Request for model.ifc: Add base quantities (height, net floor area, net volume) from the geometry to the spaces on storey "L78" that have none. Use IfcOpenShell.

First a look at what the model holds.

```python
import ifcopenshell
import ifcopenshell.util.element
import ifcopenshell.util.unit

model = ifcopenshell.open("model.ifc")
print(model.schema)
for unit_type in ("LENGTHUNIT", "AREAUNIT", "VOLUMEUNIT"):
    print(unit_type, ifcopenshell.util.unit.calculate_unit_scale(model, unit_type))
storey = next(s for s in model.by_type("IfcBuildingStorey") if s.Name == "L78")
spaces = [e for e in ifcopenshell.util.element.get_decomposition(storey) if e.is_a("IfcSpace")]
for e in sorted(spaces, key=lambda e: e.id()):
    print(e.id(), e.is_a(), e.Name, list(ifcopenshell.util.element.get_psets(e, qtos_only=True)), sep=" | ")
```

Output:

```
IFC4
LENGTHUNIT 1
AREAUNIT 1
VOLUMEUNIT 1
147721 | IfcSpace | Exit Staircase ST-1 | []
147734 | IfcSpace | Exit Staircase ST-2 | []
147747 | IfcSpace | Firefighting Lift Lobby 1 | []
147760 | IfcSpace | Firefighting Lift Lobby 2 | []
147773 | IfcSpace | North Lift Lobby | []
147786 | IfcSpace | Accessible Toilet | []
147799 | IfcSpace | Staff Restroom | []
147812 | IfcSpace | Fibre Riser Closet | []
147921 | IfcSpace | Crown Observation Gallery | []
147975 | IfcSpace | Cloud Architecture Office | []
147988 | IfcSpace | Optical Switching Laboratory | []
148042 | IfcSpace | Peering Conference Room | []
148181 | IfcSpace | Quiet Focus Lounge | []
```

```python
import ifcopenshell
import ifcopenshell.api.pset
import ifcopenshell.geom
import ifcopenshell.util.element
import ifcopenshell.util.shape
import ifcopenshell.util.unit

model = ifcopenshell.open("model.ifc")
unit_scale = ifcopenshell.util.unit.calculate_unit_scale(model)
area_scale = ifcopenshell.util.unit.calculate_unit_scale(model, "AREAUNIT")
volume_scale = ifcopenshell.util.unit.calculate_unit_scale(model, "VOLUMEUNIT")
settings = ifcopenshell.geom.settings()

storey = next(s for s in model.by_type("IfcBuildingStorey") if s.Name == "L78")
spaces = [e for e in ifcopenshell.util.element.get_decomposition(storey) if e.is_a("IfcSpace")]

for e in sorted(spaces, key=lambda e: e.id()):
    if ifcopenshell.util.element.get_psets(e, qtos_only=True, should_inherit=False):
        continue
    # Geometry comes back in metres, in the element's own axes.
    shape = ifcopenshell.geom.create_shape(settings, e)
    values = {
        "Height": ifcopenshell.util.shape.get_z(shape.geometry) / unit_scale,
        "NetFloorArea": ifcopenshell.util.shape.get_footprint_area(shape.geometry) / area_scale,
        "NetVolume": ifcopenshell.util.shape.get_volume(shape.geometry) / volume_scale,
    }
    qto = ifcopenshell.api.pset.add_qto(model, product=e, name="Qto_SpaceBaseQuantities")
    ifcopenshell.api.pset.edit_qto(model, qto=qto, properties=values)
    print(e.id(), {k: round(v, 3) for k, v in values.items()})

model.write("model_rev.ifc")
```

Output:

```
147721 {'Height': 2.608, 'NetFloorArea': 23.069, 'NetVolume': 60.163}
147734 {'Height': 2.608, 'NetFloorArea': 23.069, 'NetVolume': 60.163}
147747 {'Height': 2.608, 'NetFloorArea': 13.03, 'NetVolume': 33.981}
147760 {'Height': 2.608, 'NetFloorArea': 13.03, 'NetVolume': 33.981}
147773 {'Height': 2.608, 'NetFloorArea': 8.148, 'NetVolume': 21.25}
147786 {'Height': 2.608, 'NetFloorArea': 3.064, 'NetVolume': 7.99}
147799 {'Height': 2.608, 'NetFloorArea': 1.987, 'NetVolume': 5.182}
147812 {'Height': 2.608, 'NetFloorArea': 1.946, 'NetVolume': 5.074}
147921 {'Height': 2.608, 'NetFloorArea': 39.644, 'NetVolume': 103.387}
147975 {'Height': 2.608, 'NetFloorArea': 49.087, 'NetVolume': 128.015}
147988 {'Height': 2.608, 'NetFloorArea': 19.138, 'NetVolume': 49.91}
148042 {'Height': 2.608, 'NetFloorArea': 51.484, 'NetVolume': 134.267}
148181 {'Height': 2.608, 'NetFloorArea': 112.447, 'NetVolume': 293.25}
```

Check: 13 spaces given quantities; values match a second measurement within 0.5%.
